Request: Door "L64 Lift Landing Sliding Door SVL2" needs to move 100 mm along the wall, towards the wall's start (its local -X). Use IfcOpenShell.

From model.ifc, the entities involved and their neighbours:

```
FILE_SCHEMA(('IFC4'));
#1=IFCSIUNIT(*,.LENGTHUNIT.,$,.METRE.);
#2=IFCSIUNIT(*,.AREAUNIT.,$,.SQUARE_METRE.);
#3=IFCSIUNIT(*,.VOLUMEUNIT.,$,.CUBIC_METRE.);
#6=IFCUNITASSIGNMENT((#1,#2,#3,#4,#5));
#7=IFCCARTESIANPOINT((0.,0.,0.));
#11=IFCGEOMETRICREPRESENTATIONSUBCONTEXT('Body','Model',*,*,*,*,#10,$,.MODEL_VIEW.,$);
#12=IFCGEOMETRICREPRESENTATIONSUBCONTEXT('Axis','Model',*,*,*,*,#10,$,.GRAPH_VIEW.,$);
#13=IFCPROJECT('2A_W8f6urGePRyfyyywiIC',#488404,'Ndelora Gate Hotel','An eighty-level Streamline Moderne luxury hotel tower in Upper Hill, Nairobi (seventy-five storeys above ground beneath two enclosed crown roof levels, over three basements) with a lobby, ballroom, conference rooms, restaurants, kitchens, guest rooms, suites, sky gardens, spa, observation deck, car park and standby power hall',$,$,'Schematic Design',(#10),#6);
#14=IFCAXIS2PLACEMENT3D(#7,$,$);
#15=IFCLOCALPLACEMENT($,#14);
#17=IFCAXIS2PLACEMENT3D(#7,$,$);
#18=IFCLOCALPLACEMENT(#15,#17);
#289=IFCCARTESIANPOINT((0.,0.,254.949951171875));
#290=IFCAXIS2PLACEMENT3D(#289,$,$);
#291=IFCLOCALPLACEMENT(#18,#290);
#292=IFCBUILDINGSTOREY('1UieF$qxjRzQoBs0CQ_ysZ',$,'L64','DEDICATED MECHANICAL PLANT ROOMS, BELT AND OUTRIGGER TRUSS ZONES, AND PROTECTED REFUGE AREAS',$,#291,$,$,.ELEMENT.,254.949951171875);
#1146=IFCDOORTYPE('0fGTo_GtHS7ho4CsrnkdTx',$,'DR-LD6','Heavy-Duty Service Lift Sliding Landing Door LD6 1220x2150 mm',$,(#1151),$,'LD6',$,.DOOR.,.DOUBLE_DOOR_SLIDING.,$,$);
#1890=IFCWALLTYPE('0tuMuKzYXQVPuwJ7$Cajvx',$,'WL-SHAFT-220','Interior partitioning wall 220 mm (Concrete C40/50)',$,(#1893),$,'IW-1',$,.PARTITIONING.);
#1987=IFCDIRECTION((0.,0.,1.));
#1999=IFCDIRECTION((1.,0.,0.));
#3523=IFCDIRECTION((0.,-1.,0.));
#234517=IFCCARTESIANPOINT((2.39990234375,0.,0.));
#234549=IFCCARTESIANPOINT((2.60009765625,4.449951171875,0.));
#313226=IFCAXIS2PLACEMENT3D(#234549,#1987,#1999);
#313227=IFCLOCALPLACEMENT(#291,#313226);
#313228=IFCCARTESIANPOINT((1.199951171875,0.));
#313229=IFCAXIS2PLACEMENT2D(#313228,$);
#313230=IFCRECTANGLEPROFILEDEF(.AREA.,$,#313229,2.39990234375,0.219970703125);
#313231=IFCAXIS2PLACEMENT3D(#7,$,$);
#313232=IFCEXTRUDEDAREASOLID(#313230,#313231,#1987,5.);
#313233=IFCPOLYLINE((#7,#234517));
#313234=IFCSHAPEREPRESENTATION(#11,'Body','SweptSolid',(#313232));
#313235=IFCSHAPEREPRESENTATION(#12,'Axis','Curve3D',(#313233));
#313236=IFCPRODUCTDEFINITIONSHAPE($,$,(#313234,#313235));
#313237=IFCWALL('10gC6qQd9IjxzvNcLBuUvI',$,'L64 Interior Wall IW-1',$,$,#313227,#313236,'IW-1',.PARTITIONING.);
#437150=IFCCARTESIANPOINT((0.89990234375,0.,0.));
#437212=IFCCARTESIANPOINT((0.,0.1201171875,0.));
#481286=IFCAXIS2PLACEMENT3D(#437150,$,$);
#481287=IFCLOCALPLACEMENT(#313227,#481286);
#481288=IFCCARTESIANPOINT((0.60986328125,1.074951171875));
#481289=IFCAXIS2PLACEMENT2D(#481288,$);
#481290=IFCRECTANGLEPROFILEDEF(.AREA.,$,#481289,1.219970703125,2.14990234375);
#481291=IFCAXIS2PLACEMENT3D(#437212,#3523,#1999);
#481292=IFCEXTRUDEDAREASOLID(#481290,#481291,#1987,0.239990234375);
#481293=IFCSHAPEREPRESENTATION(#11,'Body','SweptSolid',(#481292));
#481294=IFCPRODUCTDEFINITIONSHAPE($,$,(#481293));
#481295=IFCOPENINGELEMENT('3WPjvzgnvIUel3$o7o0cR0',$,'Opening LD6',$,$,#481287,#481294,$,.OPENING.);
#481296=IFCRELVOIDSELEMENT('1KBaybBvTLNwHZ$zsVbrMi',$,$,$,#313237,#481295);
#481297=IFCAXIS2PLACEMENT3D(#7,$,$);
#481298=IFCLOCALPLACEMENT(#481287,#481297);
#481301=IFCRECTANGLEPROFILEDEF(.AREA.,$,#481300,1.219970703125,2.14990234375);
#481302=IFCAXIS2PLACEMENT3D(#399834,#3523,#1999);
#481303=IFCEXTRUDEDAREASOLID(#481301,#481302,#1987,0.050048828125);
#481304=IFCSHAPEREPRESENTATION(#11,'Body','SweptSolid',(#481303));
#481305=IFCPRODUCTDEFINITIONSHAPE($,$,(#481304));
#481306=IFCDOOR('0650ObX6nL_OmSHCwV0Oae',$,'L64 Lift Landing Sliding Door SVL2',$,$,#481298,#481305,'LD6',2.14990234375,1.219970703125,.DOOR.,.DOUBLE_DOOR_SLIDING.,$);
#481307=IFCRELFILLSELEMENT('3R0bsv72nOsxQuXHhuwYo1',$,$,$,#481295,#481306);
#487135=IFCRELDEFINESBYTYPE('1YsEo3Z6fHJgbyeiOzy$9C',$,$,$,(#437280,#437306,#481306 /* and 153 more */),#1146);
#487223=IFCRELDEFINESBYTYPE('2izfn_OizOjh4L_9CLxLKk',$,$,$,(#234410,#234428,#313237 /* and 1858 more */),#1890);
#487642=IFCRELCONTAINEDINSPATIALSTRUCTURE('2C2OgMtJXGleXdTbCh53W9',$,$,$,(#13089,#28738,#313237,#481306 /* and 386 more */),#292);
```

```python
import ifcopenshell
import ifcopenshell.api.geometry
import ifcopenshell.util.placement

model = ifcopenshell.open("model.ifc")

door = model.by_guid("0650ObX6nL_OmSHCwV0Oae")
opening = door.FillsVoids[0].RelatingOpeningElement
wall = opening.VoidsElements[0].RelatingBuildingElement

wall_matrix = ifcopenshell.util.placement.get_local_placement(wall.ObjectPlacement)
shift = wall_matrix[:3, 0] * -0.1
before = ifcopenshell.util.placement.get_local_placement(door.ObjectPlacement)[:3, 3].copy()

# The door is placed relative to its opening, so it follows when the opening moves.
matrix = ifcopenshell.util.placement.get_local_placement(opening.ObjectPlacement)
matrix[:3, 3] += shift
ifcopenshell.api.geometry.edit_object_placement(
    model, product=opening, matrix=matrix, is_si=False, should_transform_children=True
)

after = ifcopenshell.util.placement.get_local_placement(door.ObjectPlacement)[:3, 3]
print("door moved by", (after - before).round(3) + 0.0)

model.write("model-out.ifc")
```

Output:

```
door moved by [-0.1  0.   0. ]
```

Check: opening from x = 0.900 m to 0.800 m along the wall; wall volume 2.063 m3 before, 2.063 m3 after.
